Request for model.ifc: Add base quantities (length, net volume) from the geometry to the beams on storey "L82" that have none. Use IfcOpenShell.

First a look at what the model holds.

```python
import ifcopenshell
import ifcopenshell.util.element
import ifcopenshell.util.unit

model = ifcopenshell.open("model.ifc")
print(model.schema)
for unit_type in ("LENGTHUNIT", "AREAUNIT", "VOLUMEUNIT"):
    print(unit_type, ifcopenshell.util.unit.calculate_unit_scale(model, unit_type))
storey = next(s for s in model.by_type("IfcBuildingStorey") if s.Name == "L82")
beams = [e for e in ifcopenshell.util.element.get_decomposition(storey) if e.is_a("IfcBeam")]
for e in sorted(beams, key=lambda e: e.id()):
    print(e.id(), e.is_a(), e.Name, list(ifcopenshell.util.element.get_psets(e, qtos_only=True)), sep=" | ")
```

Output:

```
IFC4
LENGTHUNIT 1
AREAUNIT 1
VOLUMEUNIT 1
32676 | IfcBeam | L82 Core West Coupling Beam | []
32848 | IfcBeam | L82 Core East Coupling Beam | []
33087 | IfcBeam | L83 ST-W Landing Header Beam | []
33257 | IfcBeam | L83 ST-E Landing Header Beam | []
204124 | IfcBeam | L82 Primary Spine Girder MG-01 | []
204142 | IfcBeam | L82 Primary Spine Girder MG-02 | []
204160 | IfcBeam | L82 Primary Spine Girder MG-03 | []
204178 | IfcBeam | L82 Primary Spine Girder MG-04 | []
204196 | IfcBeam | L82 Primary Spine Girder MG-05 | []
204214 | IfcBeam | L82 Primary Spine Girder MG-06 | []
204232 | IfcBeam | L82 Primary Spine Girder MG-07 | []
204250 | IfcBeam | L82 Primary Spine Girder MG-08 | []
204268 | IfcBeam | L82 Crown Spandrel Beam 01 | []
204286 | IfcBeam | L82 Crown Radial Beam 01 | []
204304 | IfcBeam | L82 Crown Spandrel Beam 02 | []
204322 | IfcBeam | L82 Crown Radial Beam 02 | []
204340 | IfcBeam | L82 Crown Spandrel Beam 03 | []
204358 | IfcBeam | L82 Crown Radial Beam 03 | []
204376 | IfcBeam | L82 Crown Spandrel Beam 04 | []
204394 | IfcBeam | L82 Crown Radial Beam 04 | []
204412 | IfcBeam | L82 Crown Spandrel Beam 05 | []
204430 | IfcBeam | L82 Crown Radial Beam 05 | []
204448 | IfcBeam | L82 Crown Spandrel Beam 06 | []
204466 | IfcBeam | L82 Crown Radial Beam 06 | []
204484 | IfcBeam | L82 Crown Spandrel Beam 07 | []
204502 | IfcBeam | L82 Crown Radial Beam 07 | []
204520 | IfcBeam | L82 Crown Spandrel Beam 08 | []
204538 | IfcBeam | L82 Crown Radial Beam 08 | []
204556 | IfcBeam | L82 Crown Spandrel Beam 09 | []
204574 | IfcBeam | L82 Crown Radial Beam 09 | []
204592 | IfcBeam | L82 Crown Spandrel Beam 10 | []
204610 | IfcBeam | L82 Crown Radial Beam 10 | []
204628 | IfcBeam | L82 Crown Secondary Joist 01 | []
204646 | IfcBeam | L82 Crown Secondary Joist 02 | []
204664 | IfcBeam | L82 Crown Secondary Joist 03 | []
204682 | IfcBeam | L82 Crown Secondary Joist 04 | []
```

```python
import ifcopenshell
import ifcopenshell.api.pset
import ifcopenshell.geom
import ifcopenshell.util.element
import ifcopenshell.util.shape
import ifcopenshell.util.unit

model = ifcopenshell.open("model.ifc")
unit_scale = ifcopenshell.util.unit.calculate_unit_scale(model)
volume_scale = ifcopenshell.util.unit.calculate_unit_scale(model, "VOLUMEUNIT")
settings = ifcopenshell.geom.settings()

storey = next(s for s in model.by_type("IfcBuildingStorey") if s.Name == "L82")
beams = [e for e in ifcopenshell.util.element.get_decomposition(storey) if e.is_a("IfcBeam")]

for e in sorted(beams, key=lambda e: e.id()):
    if ifcopenshell.util.element.get_psets(e, qtos_only=True, should_inherit=False):
        continue
    # Geometry comes back in metres, in the element's own axes.
    shape = ifcopenshell.geom.create_shape(settings, e)
    values = {
        "Length": ifcopenshell.util.shape.get_max_xyz(shape.geometry) / unit_scale,
        "NetVolume": ifcopenshell.util.shape.get_volume(shape.geometry) / volume_scale,
    }
    qto = ifcopenshell.api.pset.add_qto(model, product=e, name="Qto_BeamBaseQuantities")
    ifcopenshell.api.pset.edit_qto(model, qto=qto, properties=values)
    print(e.id(), {k: round(v, 3) for k, v in values.items()})

model.write("model_updated.ifc")
```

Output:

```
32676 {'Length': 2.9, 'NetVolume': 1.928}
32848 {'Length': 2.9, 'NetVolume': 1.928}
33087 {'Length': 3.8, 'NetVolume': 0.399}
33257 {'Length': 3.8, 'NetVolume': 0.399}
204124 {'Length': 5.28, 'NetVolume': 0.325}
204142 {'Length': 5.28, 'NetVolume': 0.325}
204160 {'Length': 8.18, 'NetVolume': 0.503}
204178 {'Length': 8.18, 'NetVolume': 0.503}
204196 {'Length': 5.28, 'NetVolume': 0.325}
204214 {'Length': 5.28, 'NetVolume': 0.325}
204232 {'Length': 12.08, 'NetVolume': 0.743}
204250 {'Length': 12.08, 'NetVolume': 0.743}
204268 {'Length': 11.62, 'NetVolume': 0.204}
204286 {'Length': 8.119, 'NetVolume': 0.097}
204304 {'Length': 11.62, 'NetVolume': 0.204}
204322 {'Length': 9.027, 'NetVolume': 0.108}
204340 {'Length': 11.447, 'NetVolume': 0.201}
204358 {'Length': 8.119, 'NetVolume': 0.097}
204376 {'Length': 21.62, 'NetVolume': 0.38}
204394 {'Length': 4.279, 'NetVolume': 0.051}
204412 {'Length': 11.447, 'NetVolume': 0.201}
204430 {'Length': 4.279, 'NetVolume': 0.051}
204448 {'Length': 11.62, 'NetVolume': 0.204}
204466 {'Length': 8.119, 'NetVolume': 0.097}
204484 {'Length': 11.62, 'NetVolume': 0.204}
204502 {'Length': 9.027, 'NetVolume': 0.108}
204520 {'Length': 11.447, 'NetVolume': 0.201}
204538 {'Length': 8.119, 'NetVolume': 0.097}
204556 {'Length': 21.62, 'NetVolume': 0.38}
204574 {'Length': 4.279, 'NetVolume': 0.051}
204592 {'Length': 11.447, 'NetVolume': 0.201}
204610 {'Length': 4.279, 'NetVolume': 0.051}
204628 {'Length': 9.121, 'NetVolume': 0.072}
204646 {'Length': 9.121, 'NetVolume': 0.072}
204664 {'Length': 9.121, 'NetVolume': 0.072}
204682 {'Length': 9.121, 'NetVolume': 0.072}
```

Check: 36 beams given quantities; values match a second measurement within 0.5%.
